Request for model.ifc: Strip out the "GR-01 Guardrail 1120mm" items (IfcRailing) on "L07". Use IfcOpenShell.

First a look at what the model holds.

```python
import ifcopenshell
import ifcopenshell.util.element

model = ifcopenshell.open("model.ifc")
print(model.schema)
storey = next(s for s in model.by_type("IfcBuildingStorey") if s.Name == "L07")
railings = [e for e in ifcopenshell.util.element.get_decomposition(storey) if e.is_a("IfcRailing")]
seen = {}
for e in railings:
    element_type = ifcopenshell.util.element.get_type(e)
    name = element_type.Name if element_type not in (None, e) else None
    seen[name] = seen.get(name, 0) + 1
for name, count in sorted(seen.items(), key=str):
    print(count, "x", name)
```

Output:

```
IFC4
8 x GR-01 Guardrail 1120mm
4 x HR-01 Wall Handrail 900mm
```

```python
import ifcopenshell
import ifcopenshell.api.root
import ifcopenshell.util.element

model = ifcopenshell.open("model.ifc")

storey = next(s for s in model.by_type("IfcBuildingStorey") if s.Name == "L07")
railings = [e for e in ifcopenshell.util.element.get_decomposition(storey) if e.is_a("IfcRailing")]
targets = [e for e in railings if (t := ifcopenshell.util.element.get_type(e)) not in (None, e) and t.Name == "GR-01 Guardrail 1120mm"]

for e in targets:
    ifcopenshell.api.root.remove_product(model, product=e)
print(len(targets), "removed")

model.write("model_rev.ifc")
```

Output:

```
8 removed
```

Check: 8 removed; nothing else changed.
